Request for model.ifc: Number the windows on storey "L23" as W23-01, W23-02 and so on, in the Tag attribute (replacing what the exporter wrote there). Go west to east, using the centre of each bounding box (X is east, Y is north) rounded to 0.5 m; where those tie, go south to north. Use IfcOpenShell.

First a look at what the model holds.

```python
import ifcopenshell
import ifcopenshell.util.element
import ifcopenshell.util.placement

model = ifcopenshell.open("model.ifc")
print(model.schema)
storey = next(s for s in model.by_type("IfcBuildingStorey") if s.Name == "L23")
windows = [e for e in ifcopenshell.util.element.get_decomposition(storey) if e.is_a("IfcWindow")]
for e in sorted(windows, key=lambda e: e.id()):
    origin = ifcopenshell.util.placement.get_local_placement(e.ObjectPlacement)[:3, 3]
    print(e.id(), e.Tag, e.Name, origin.round(2) + 0.0, sep=" | ")
```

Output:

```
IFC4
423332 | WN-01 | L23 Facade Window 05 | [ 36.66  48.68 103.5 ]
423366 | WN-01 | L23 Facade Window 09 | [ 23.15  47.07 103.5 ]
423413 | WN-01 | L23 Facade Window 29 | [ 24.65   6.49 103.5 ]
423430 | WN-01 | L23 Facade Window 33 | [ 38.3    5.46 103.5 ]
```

```python
import ifcopenshell
import ifcopenshell.geom
import ifcopenshell.util.element
import ifcopenshell.util.shape

model = ifcopenshell.open("model.ifc")
settings = ifcopenshell.geom.settings()
settings.set("use-world-coords", True)


def centre(element):
    shape = ifcopenshell.geom.create_shape(settings, element)
    return ifcopenshell.util.shape.get_bbox_centroid(shape.geometry)


storey = next(s for s in model.by_type("IfcBuildingStorey") if s.Name == "L23")
windows = [e for e in ifcopenshell.util.element.get_decomposition(storey) if e.is_a("IfcWindow")]

# Insertion points can sit at a corner or the storey origin, so sort by the geometry (in metres).
centres = {e: centre(e) for e in windows}
windows.sort(key=lambda e: (round(centres[e][0] / 0.5), centres[e][1]))

for i, e in enumerate(windows, start=1):
    number = f"W23-{i:02d}"
    e.Tag = number
    print(e.id(), number)

model.write("model-out.ifc")
```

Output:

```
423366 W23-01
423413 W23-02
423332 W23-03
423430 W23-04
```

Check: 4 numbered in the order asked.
